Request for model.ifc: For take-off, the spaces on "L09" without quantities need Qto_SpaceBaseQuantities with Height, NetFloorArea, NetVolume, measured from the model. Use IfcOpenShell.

First a look at what the model holds.

```python
import ifcopenshell
import ifcopenshell.util.element
import ifcopenshell.util.unit

model = ifcopenshell.open("model.ifc")
print(model.schema)
for unit_type in ("LENGTHUNIT", "AREAUNIT", "VOLUMEUNIT"):
    print(unit_type, ifcopenshell.util.unit.calculate_unit_scale(model, unit_type))
storey = next(s for s in model.by_type("IfcBuildingStorey") if s.Name == "L09")
spaces = [e for e in ifcopenshell.util.element.get_decomposition(storey) if e.is_a("IfcSpace")]
for e in sorted(spaces, key=lambda e: e.id()):
    print(e.id(), e.is_a(), e.Name, list(ifcopenshell.util.element.get_psets(e, qtos_only=True)), sep=" | ")
```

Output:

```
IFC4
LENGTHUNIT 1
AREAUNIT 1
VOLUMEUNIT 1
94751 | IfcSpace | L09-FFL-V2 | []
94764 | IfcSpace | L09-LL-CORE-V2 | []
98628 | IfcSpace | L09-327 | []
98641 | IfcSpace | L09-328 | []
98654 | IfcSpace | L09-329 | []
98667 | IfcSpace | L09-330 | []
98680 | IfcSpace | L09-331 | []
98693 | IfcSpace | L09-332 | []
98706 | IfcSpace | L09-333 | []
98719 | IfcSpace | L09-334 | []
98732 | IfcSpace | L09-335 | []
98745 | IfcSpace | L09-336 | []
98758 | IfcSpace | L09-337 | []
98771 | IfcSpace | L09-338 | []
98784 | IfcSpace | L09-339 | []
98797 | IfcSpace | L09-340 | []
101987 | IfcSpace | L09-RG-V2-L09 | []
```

```python
import ifcopenshell
import ifcopenshell.api.pset
import ifcopenshell.geom
import ifcopenshell.util.element
import ifcopenshell.util.shape
import ifcopenshell.util.unit

model = ifcopenshell.open("model.ifc")
unit_scale = ifcopenshell.util.unit.calculate_unit_scale(model)
area_scale = ifcopenshell.util.unit.calculate_unit_scale(model, "AREAUNIT")
volume_scale = ifcopenshell.util.unit.calculate_unit_scale(model, "VOLUMEUNIT")
settings = ifcopenshell.geom.settings()

storey = next(s for s in model.by_type("IfcBuildingStorey") if s.Name == "L09")
spaces = [e for e in ifcopenshell.util.element.get_decomposition(storey) if e.is_a("IfcSpace")]

for e in sorted(spaces, key=lambda e: e.id()):
    if ifcopenshell.util.element.get_psets(e, qtos_only=True, should_inherit=False):
        continue
    # Geometry comes back in metres, in the element's own axes.
    shape = ifcopenshell.geom.create_shape(settings, e)
    values = {
        "Height": ifcopenshell.util.shape.get_z(shape.geometry) / unit_scale,
        "NetFloorArea": ifcopenshell.util.shape.get_footprint_area(shape.geometry) / area_scale,
        "NetVolume": ifcopenshell.util.shape.get_volume(shape.geometry) / volume_scale,
    }
    qto = ifcopenshell.api.pset.add_qto(model, product=e, name="Qto_SpaceBaseQuantities")
    ifcopenshell.api.pset.edit_qto(model, qto=qto, properties=values)
    print(e.id(), {k: round(v, 3) for k, v in values.items()})

model.write("model-out.ifc")
```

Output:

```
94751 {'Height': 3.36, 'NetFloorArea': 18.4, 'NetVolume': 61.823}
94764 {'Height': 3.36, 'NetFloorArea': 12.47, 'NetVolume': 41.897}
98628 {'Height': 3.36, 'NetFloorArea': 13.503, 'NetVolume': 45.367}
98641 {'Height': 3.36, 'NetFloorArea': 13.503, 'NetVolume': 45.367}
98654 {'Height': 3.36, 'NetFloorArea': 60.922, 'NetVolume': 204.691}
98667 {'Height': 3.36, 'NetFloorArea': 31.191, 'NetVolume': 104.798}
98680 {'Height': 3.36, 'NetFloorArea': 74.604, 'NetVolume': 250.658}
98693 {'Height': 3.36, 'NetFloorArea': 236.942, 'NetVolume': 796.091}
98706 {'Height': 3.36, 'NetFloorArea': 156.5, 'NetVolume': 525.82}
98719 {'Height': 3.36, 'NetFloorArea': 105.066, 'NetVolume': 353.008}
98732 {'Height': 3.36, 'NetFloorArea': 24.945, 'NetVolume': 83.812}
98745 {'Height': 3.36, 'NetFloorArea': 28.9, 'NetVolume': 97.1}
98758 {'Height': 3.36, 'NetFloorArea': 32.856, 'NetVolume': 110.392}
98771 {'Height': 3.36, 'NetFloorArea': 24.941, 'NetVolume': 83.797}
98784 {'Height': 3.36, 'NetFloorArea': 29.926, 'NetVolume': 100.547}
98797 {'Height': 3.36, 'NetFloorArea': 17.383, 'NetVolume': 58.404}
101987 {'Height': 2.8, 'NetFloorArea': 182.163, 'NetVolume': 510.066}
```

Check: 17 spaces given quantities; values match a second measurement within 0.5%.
